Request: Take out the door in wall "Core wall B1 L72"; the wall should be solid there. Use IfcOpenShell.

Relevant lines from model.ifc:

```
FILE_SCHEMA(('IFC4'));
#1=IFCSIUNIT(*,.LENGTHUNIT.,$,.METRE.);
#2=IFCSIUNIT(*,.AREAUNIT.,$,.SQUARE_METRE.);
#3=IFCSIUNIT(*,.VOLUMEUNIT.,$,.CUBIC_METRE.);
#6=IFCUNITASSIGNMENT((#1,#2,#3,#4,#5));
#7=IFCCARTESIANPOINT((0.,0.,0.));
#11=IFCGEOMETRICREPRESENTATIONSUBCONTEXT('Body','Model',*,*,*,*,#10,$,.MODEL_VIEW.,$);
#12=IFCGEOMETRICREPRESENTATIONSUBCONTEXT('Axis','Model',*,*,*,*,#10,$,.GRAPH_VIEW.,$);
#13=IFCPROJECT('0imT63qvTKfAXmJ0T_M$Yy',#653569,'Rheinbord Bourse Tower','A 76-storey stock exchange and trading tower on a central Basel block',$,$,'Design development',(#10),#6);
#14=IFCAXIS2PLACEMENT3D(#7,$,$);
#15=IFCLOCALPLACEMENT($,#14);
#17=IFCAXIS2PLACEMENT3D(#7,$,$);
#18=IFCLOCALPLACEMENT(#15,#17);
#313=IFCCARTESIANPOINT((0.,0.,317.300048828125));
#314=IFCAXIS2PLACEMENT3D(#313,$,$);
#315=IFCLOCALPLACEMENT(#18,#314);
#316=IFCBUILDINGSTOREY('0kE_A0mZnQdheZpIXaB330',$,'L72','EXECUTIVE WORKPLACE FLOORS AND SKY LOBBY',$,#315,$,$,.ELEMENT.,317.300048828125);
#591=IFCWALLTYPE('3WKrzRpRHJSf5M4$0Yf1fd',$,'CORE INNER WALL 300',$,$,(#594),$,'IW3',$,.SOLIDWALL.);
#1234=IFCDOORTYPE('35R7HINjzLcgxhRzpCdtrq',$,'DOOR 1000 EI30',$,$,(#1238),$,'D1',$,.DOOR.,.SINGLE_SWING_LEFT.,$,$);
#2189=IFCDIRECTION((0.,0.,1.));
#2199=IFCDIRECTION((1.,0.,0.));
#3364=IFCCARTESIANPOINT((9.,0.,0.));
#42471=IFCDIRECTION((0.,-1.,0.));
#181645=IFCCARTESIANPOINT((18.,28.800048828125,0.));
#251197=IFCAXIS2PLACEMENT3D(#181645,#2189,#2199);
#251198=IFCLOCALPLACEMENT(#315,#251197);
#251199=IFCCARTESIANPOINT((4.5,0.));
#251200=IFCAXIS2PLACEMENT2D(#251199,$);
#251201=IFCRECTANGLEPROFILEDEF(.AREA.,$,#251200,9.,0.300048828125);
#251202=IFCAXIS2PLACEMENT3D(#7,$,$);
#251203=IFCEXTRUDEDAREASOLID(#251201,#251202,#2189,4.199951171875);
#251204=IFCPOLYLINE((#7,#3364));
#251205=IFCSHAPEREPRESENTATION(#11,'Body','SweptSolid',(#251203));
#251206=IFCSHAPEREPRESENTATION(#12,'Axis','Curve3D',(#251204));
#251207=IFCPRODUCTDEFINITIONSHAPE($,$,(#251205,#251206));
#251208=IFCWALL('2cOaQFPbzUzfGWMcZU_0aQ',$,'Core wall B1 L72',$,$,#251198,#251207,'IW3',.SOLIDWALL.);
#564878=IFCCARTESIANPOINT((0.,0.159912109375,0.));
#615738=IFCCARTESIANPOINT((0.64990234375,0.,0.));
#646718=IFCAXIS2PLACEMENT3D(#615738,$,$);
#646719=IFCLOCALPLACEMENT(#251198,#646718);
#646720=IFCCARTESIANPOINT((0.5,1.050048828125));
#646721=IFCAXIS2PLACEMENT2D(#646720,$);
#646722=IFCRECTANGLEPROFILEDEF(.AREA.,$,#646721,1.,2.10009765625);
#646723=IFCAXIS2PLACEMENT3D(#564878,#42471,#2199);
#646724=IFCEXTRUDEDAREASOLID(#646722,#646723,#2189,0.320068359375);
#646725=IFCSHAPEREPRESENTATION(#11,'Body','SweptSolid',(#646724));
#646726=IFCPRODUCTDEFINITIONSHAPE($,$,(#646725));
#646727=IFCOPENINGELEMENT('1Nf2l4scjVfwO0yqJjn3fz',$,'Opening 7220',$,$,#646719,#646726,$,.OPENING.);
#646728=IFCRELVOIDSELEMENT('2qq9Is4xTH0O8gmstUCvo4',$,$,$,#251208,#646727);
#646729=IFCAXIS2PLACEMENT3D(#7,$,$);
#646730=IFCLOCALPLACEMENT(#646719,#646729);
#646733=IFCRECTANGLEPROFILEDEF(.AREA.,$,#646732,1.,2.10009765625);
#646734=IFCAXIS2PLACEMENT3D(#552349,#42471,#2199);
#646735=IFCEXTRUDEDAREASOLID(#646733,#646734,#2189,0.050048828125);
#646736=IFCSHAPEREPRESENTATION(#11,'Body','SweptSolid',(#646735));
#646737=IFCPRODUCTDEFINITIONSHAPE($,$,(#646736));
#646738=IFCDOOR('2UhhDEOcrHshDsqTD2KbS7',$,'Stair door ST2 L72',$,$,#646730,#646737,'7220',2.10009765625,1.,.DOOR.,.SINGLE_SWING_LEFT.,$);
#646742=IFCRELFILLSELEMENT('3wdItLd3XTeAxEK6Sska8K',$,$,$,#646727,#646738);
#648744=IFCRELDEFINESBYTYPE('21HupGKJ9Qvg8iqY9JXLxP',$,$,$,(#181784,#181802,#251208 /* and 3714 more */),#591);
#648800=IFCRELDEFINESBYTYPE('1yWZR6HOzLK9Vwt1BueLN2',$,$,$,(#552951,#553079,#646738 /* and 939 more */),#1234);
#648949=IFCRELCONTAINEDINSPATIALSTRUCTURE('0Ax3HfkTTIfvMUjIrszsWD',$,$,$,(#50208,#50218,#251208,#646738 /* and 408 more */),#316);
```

```python
import ifcopenshell
import ifcopenshell.api.feature
import ifcopenshell.api.root
import ifcopenshell.geom
import ifcopenshell.util.shape

model = ifcopenshell.open("model.ifc")
settings = ifcopenshell.geom.settings()


def volume(element):
    """Net volume in cubic metres, openings subtracted."""
    shape = ifcopenshell.geom.create_shape(settings, element)
    return ifcopenshell.util.shape.get_volume(shape.geometry)


door = model.by_guid("2UhhDEOcrHshDsqTD2KbS7")
opening = door.FillsVoids[0].RelatingOpeningElement
wall = opening.VoidsElements[0].RelatingBuildingElement
before = volume(wall)

ifcopenshell.api.root.remove_product(model, product=door)
ifcopenshell.api.feature.remove_feature(model, feature=opening)

after = volume(wall)

print(f"wall volume {before:.3f} -> {after:.3f} m3")

model.write("model_v2.ifc")
```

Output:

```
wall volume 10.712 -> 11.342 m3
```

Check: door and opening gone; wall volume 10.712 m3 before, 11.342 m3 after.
